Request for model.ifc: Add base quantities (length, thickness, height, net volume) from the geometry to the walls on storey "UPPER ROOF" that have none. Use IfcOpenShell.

First a look at what the model holds.

```python
import ifcopenshell
import ifcopenshell.util.element
import ifcopenshell.util.unit

model = ifcopenshell.open("model.ifc")
print(model.schema)
for unit_type in ("LENGTHUNIT", "AREAUNIT", "VOLUMEUNIT"):
    print(unit_type, ifcopenshell.util.unit.calculate_unit_scale(model, unit_type))
storey = next(s for s in model.by_type("IfcBuildingStorey") if s.Name == "UPPER ROOF")
walls = [e for e in ifcopenshell.util.element.get_decomposition(storey) if e.is_a("IfcWall")]
for e in sorted(walls, key=lambda e: e.id()):
    print(e.id(), e.is_a(), e.Name, list(ifcopenshell.util.element.get_psets(e, qtos_only=True)), sep=" | ")
```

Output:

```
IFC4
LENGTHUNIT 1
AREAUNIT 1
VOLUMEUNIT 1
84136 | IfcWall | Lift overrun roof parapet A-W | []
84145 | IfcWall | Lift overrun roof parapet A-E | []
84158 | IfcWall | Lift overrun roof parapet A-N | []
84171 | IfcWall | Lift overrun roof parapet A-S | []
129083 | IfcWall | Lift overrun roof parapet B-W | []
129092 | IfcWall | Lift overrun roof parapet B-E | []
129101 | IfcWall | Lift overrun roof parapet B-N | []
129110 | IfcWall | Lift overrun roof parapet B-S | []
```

```python
import ifcopenshell
import ifcopenshell.api.pset
import ifcopenshell.geom
import ifcopenshell.util.element
import ifcopenshell.util.shape
import ifcopenshell.util.unit

model = ifcopenshell.open("model.ifc")
unit_scale = ifcopenshell.util.unit.calculate_unit_scale(model)
volume_scale = ifcopenshell.util.unit.calculate_unit_scale(model, "VOLUMEUNIT")
settings = ifcopenshell.geom.settings()

storey = next(s for s in model.by_type("IfcBuildingStorey") if s.Name == "UPPER ROOF")
walls = [e for e in ifcopenshell.util.element.get_decomposition(storey) if e.is_a("IfcWall")]

for e in sorted(walls, key=lambda e: e.id()):
    if ifcopenshell.util.element.get_psets(e, qtos_only=True, should_inherit=False):
        continue
    # Geometry comes back in metres, in the element's own axes.
    shape = ifcopenshell.geom.create_shape(settings, e)
    values = {
        "Length": ifcopenshell.util.shape.get_x(shape.geometry) / unit_scale,
        "Width": ifcopenshell.util.shape.get_y(shape.geometry) / unit_scale,
        "Height": ifcopenshell.util.shape.get_z(shape.geometry) / unit_scale,
        "NetVolume": ifcopenshell.util.shape.get_volume(shape.geometry) / volume_scale,
    }
    qto = ifcopenshell.api.pset.add_qto(model, product=e, name="Qto_WallBaseQuantities")
    ifcopenshell.api.pset.edit_qto(model, qto=qto, properties=values)
    print(e.id(), {k: round(v, 3) for k, v in values.items()})

model.write("model_edited.ifc")
```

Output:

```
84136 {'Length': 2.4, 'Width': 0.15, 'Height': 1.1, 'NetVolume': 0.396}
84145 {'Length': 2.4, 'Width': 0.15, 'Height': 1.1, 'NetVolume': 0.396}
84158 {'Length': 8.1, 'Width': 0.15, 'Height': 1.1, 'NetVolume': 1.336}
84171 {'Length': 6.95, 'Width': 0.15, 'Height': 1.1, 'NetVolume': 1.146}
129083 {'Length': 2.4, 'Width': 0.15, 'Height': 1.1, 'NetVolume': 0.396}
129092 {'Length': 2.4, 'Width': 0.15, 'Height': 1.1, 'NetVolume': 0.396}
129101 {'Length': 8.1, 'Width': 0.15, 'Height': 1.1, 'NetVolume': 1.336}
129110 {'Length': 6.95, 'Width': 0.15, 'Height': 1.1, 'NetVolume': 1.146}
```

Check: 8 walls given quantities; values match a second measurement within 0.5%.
